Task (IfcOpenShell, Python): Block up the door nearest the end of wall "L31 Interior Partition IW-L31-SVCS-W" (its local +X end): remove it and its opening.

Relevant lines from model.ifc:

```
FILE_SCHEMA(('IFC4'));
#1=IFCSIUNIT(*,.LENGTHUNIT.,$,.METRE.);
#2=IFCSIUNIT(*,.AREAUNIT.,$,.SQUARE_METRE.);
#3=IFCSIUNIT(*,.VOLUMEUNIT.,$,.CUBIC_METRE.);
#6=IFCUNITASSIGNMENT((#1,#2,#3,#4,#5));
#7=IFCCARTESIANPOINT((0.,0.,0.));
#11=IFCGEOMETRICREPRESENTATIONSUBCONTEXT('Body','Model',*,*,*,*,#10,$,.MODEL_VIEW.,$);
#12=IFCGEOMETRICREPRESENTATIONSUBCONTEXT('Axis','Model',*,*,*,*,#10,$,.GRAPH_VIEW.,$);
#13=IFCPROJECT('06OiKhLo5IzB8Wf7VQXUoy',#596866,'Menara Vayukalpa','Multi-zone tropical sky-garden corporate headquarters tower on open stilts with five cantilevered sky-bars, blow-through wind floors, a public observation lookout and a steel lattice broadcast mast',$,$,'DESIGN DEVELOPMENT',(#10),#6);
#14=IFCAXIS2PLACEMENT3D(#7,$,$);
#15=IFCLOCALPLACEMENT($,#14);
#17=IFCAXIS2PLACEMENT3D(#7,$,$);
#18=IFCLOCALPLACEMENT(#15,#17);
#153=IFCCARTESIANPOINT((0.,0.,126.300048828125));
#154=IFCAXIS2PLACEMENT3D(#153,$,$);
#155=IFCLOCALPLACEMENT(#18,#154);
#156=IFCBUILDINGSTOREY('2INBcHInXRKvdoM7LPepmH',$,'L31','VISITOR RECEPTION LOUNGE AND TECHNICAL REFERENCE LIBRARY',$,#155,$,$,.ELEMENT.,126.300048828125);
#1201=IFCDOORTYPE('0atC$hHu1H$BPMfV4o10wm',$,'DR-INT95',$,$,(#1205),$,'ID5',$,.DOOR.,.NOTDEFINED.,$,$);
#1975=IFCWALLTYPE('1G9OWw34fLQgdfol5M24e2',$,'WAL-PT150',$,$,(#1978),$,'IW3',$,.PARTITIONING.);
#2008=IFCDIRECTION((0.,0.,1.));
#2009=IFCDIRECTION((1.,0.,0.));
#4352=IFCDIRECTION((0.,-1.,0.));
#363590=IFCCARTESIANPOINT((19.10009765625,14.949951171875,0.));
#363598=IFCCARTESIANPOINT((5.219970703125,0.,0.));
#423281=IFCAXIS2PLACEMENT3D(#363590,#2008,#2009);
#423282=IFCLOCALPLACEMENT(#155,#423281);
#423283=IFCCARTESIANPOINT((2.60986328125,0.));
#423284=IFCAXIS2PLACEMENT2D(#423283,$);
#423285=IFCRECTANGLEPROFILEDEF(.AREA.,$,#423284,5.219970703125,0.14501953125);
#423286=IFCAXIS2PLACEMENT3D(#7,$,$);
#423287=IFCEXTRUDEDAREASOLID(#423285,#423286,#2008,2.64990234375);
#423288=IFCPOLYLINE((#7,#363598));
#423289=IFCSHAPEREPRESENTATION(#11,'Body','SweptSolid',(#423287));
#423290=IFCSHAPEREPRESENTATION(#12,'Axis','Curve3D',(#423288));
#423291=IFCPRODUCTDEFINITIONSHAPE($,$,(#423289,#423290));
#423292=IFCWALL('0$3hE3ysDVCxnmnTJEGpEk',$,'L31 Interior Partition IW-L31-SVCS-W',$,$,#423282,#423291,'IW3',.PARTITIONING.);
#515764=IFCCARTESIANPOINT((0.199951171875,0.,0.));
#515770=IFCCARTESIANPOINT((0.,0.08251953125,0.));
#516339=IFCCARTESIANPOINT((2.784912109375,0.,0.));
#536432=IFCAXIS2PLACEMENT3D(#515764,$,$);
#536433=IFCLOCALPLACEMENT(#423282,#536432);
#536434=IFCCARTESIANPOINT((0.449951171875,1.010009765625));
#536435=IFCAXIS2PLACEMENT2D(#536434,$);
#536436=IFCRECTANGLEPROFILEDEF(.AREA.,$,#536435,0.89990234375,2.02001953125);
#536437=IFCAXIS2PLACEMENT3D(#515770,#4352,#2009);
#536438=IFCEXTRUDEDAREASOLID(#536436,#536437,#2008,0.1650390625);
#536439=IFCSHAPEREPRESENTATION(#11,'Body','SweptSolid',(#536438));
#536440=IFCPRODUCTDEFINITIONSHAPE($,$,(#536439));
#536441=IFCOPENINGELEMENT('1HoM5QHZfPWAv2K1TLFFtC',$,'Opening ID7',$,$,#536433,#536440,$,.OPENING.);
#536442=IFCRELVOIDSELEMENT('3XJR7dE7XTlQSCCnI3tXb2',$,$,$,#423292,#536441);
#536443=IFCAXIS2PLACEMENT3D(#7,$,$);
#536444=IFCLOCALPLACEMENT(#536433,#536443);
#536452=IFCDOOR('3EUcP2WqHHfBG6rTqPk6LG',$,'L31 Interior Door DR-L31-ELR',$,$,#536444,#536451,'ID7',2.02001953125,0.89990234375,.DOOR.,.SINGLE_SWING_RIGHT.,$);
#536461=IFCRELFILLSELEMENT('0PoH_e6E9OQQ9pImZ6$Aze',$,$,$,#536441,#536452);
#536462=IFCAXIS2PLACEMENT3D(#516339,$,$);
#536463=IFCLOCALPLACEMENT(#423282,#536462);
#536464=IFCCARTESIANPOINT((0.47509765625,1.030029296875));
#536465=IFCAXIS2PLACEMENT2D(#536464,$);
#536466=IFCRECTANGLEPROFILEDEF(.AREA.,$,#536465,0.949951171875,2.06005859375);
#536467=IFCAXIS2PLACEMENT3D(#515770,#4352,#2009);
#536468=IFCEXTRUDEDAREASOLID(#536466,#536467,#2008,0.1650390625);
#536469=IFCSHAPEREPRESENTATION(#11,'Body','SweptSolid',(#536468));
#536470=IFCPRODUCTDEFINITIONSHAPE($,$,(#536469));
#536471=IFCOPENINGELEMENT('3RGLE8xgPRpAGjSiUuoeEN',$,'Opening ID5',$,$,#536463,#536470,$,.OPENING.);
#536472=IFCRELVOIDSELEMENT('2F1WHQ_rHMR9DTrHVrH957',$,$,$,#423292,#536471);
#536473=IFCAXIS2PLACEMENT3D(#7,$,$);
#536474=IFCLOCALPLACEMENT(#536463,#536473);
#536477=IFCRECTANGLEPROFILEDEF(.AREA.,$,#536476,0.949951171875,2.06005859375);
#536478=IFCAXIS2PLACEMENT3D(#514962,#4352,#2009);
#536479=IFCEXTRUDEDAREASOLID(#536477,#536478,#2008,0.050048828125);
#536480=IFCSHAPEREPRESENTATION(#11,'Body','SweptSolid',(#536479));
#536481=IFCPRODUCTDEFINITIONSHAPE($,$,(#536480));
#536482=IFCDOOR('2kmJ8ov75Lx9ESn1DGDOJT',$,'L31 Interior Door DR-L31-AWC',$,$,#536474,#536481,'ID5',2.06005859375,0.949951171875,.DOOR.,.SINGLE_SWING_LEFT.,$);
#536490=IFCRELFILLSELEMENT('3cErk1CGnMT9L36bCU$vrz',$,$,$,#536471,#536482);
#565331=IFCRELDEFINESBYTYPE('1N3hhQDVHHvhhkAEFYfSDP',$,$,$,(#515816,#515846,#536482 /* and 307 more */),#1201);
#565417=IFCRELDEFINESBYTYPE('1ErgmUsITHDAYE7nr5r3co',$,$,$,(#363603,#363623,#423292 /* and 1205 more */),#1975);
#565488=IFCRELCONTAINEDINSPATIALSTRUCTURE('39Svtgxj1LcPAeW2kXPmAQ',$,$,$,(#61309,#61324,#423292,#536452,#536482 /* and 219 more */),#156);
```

```python
import ifcopenshell
import ifcopenshell.api.feature
import ifcopenshell.api.root
import ifcopenshell.geom
import ifcopenshell.util.shape

model = ifcopenshell.open("model.ifc")
settings = ifcopenshell.geom.settings()


def volume(element):
    """Net volume in cubic metres, openings subtracted."""
    shape = ifcopenshell.geom.create_shape(settings, element)
    return ifcopenshell.util.shape.get_volume(shape.geometry)


door = model.by_id(536482)
opening = door.FillsVoids[0].RelatingOpeningElement
wall = opening.VoidsElements[0].RelatingBuildingElement
before = volume(wall)

ifcopenshell.api.root.remove_product(model, product=door)
ifcopenshell.api.feature.remove_feature(model, feature=opening)

after = volume(wall)

print(f"wall volume {before:.3f} -> {after:.3f} m3")

model.write("model-out.ifc")
```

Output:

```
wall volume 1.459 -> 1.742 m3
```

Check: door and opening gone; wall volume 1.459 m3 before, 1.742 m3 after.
